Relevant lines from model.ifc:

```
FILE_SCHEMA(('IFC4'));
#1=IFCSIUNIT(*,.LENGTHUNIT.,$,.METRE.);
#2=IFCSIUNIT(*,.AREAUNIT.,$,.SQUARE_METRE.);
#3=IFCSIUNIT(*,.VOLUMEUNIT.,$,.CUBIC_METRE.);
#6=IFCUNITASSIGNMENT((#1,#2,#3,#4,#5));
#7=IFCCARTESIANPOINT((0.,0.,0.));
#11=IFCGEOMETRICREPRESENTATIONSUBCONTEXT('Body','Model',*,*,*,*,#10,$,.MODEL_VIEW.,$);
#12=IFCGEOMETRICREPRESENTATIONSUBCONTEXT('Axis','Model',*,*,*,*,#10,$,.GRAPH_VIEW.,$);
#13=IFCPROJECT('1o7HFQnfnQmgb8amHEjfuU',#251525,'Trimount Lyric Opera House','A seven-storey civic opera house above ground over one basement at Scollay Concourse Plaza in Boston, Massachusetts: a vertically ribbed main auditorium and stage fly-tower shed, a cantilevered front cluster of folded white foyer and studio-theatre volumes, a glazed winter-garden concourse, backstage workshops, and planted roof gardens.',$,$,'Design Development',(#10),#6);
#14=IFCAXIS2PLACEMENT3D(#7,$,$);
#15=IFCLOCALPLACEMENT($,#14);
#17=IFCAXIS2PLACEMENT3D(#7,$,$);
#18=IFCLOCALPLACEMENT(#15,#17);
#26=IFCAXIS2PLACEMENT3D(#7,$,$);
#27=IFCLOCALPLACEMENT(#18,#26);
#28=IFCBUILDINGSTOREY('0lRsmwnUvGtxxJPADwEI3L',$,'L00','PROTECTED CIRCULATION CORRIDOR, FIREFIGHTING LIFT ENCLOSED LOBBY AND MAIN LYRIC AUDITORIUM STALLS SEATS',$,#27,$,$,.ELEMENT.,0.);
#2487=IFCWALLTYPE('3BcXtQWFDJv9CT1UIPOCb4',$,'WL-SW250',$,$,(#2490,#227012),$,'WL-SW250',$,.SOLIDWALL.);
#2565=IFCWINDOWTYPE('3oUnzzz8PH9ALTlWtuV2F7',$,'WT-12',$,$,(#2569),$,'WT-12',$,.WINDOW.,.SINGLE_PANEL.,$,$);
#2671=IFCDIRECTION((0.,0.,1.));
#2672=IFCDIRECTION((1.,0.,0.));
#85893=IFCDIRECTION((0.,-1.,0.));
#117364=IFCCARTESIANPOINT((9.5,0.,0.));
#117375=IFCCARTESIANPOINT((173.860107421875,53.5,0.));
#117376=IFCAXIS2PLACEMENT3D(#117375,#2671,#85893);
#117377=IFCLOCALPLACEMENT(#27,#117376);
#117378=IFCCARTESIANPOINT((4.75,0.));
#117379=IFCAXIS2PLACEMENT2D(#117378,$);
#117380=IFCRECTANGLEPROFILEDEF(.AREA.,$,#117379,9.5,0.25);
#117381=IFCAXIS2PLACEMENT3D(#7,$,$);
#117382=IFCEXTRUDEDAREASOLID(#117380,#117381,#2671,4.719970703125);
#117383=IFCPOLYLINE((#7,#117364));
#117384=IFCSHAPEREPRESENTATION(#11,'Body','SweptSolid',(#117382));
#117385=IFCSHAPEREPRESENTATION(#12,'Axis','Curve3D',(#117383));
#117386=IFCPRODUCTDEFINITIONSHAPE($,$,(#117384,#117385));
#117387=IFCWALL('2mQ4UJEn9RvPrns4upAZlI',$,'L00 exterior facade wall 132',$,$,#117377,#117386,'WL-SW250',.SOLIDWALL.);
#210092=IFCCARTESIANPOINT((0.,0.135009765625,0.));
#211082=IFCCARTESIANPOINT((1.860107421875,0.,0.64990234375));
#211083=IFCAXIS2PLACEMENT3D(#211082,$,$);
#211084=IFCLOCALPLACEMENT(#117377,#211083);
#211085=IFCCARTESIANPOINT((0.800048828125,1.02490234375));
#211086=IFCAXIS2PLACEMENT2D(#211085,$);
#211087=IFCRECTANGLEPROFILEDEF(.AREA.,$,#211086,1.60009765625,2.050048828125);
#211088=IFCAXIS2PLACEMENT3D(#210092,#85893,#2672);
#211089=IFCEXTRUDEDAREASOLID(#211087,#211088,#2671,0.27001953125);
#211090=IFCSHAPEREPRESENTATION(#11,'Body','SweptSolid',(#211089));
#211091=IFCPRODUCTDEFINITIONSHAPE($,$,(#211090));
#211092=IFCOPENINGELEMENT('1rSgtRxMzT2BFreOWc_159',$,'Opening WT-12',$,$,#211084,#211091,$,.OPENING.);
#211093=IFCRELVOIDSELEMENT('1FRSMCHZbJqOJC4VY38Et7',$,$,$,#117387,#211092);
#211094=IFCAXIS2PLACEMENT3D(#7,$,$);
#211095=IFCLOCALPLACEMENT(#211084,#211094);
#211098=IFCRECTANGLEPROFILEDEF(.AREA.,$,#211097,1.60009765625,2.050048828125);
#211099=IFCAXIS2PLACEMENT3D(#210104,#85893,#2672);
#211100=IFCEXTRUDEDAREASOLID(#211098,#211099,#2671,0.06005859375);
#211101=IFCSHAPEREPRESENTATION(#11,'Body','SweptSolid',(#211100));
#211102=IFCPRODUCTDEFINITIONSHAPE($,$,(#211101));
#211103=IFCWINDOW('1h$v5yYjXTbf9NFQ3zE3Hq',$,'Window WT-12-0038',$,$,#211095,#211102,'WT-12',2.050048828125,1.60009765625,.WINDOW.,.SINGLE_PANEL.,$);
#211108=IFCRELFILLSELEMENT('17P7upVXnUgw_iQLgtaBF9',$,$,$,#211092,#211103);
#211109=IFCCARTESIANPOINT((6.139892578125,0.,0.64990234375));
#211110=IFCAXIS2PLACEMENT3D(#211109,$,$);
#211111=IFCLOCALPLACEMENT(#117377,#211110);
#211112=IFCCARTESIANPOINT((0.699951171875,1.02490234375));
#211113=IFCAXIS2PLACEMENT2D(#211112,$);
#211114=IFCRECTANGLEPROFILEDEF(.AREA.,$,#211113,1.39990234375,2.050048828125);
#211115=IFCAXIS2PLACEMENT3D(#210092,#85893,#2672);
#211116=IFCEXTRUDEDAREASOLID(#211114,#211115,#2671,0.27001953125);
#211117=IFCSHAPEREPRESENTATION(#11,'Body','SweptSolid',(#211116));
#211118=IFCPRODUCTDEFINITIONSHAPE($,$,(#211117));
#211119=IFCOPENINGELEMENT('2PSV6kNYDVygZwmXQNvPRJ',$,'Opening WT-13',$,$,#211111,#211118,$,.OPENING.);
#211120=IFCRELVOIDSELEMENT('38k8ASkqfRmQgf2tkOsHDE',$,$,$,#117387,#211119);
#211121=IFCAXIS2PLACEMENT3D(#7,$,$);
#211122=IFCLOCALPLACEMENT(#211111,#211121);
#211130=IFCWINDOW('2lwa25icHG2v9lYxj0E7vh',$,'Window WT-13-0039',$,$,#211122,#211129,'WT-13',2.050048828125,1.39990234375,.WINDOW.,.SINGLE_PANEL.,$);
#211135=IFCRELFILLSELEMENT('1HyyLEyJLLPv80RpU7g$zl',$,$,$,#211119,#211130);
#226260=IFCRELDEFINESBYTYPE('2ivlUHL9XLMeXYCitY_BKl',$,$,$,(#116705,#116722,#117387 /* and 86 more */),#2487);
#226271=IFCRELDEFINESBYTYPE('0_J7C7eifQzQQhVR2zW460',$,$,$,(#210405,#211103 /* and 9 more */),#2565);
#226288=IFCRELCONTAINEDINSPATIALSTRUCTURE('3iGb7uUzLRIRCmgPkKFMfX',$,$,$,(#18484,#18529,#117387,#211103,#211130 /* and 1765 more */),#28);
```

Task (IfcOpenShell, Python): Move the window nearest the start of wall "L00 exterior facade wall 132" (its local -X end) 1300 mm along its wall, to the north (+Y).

```python
import ifcopenshell
import ifcopenshell.api.geometry
import ifcopenshell.util.placement
import ifcopenshell.util.unit

model = ifcopenshell.open("model.ifc")
unit_scale = ifcopenshell.util.unit.calculate_unit_scale(model)

window = model.by_guid("1h$v5yYjXTbf9NFQ3zE3Hq")
opening = window.FillsVoids[0].RelatingOpeningElement
wall = opening.VoidsElements[0].RelatingBuildingElement

wall_matrix = ifcopenshell.util.placement.get_local_placement(wall.ObjectPlacement)
shift = wall_matrix[:3, 0] * -1.3 / unit_scale
before = ifcopenshell.util.placement.get_local_placement(window.ObjectPlacement)[:3, 3].copy()

# The window is placed relative to its opening, so it follows when the opening moves.
matrix = ifcopenshell.util.placement.get_local_placement(opening.ObjectPlacement)
matrix[:3, 3] += shift
ifcopenshell.api.geometry.edit_object_placement(
    model, product=opening, matrix=matrix, is_si=False, should_transform_children=True
)

after = ifcopenshell.util.placement.get_local_placement(window.ObjectPlacement)[:3, 3]
print("window moved by", (after - before).round(3) + 0.0)

model.write("model_rev.ifc")
```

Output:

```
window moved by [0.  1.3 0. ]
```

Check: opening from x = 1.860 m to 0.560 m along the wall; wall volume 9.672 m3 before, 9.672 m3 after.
